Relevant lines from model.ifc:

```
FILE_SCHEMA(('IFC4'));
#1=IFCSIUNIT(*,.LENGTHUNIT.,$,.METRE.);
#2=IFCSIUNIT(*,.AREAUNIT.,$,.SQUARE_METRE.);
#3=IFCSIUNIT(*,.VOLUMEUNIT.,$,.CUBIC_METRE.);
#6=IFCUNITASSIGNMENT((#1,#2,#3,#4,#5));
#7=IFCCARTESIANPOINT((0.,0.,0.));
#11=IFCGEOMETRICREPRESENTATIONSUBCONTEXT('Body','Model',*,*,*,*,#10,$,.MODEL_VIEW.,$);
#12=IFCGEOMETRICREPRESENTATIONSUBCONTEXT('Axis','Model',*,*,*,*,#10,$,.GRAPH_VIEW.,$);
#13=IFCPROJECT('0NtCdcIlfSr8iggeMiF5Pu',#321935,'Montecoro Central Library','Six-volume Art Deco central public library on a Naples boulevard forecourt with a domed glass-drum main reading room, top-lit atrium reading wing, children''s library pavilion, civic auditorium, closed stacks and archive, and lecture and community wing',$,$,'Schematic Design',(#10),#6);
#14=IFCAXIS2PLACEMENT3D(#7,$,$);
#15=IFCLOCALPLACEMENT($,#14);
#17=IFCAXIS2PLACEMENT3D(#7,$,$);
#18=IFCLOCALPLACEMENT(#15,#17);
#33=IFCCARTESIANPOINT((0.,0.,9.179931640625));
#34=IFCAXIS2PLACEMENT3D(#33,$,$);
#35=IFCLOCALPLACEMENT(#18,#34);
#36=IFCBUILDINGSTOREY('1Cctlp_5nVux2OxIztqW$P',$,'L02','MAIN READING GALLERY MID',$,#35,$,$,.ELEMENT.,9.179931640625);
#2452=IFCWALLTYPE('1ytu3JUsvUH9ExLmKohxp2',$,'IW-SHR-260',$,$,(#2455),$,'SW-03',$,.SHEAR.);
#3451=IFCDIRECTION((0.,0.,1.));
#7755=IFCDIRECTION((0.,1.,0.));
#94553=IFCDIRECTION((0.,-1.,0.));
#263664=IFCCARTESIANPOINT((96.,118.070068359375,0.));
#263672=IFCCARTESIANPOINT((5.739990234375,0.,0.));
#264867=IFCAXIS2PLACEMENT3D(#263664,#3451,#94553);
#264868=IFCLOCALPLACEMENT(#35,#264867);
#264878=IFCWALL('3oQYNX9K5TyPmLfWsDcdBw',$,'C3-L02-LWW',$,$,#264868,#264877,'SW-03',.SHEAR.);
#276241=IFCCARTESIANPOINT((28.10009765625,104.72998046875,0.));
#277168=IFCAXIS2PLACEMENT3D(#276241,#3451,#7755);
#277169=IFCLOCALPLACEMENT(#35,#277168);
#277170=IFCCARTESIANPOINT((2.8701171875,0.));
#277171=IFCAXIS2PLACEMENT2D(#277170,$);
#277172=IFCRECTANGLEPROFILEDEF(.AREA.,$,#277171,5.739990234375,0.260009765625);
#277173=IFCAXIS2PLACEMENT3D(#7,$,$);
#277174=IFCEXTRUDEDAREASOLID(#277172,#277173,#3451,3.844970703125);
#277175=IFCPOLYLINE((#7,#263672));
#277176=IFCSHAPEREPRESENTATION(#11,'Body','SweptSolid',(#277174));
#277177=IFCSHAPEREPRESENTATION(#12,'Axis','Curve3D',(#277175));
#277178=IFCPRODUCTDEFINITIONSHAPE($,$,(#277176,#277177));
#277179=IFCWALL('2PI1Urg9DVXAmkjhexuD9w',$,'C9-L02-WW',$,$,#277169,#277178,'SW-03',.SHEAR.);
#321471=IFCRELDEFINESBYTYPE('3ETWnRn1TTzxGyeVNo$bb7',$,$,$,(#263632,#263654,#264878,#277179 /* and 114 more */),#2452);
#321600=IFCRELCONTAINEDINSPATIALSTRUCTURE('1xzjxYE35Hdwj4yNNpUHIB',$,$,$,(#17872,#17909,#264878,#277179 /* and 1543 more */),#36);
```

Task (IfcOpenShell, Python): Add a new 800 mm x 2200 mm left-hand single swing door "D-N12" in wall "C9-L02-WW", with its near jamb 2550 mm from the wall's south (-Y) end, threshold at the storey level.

```python
import numpy as np
import ifcopenshell
import ifcopenshell.api.feature
import ifcopenshell.api.geometry
import ifcopenshell.api.root
import ifcopenshell.api.spatial
import ifcopenshell.geom
import ifcopenshell.util.element
import ifcopenshell.util.placement
import ifcopenshell.util.representation
import ifcopenshell.util.shape
import ifcopenshell.util.unit

model = ifcopenshell.open("model.ifc")
unit_scale = ifcopenshell.util.unit.calculate_unit_scale(model)
settings = ifcopenshell.geom.settings()


def volume(element):
    """Net volume in cubic metres, openings subtracted."""
    shape = ifcopenshell.geom.create_shape(settings, element)
    return ifcopenshell.util.shape.get_volume(shape.geometry)


wall = model.by_id(277179)
storey = ifcopenshell.util.element.get_container(wall, ifc_class="IfcBuildingStorey")
context = ifcopenshell.util.representation.get_context(model, "Model", "Body", "MODEL_VIEW")
before = volume(wall)

width, height, from_end, sill = 0.8, 2.2, 2.55, 0.0  # metres

# The wall runs along its own X axis, and the end named is its -X end.
wall_shape = ifcopenshell.geom.create_shape(settings, wall)
x, y, z = ifcopenshell.util.shape.get_vertices(wall_shape.geometry).T
start = x.min() + from_end
face, thickness = float(y.min()), float(y.max() - y.min())
wall_matrix = ifcopenshell.util.placement.get_local_placement(wall.ObjectPlacement)
level = ifcopenshell.util.placement.get_local_placement(storey.ObjectPlacement)[2, 3]


def in_wall(x, y):
    """Placement at x, y metres in the wall's axes, at sill height."""
    matrix = wall_matrix.copy()
    matrix[:, 3] = wall_matrix @ np.array([x / unit_scale, y / unit_scale, 0.0, 1.0])
    matrix[2, 3] = level + sill / unit_scale
    return matrix


# Opening: a box that overshoots both wall faces by 50 mm.
opening = ifcopenshell.api.root.create_entity(model, ifc_class="IfcOpeningElement", predefined_type="OPENING")
box = ifcopenshell.api.geometry.add_wall_representation(
    model, context=context, length=width, height=height, thickness=thickness + 0.1
)
ifcopenshell.api.geometry.assign_representation(model, product=opening, representation=box)
ifcopenshell.api.geometry.edit_object_placement(model, product=opening, matrix=in_wall(start, face - 0.05), is_si=False)
ifcopenshell.api.feature.add_feature(model, feature=opening, element=wall)

door = ifcopenshell.api.root.create_entity(model, ifc_class="IfcDoor", name="D-N12", predefined_type="DOOR")
door.OverallWidth, door.OverallHeight = width / unit_scale, height / unit_scale
door.OperationType = "SINGLE_SWING_LEFT"
body = ifcopenshell.api.geometry.add_door_representation(
    model,
    context=context,
    overall_width=door.OverallWidth,
    overall_height=door.OverallHeight,
    operation_type="SINGLE_SWING_LEFT",
    lining_properties={"LiningDepth": thickness / unit_scale, "ThresholdDepth": thickness / unit_scale},
)
ifcopenshell.api.geometry.assign_representation(model, product=door, representation=body)
ifcopenshell.api.spatial.assign_container(model, products=[door], relating_structure=storey)
ifcopenshell.api.feature.add_filling(model, opening=opening, element=door)

# The lining spans the wall, so the door starts at the wall face.
ifcopenshell.api.geometry.edit_object_placement(model, product=door, matrix=in_wall(start, face), is_si=False)

after = volume(wall)

print(f"wall volume {before:.3f} -> {after:.3f} m3")

model.write("model_edited.ifc")
```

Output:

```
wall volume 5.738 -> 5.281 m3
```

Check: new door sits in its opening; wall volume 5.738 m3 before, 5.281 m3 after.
